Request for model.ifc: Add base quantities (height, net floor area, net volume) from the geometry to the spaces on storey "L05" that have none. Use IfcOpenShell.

First a look at what the model holds.

```python
import ifcopenshell
import ifcopenshell.util.element
import ifcopenshell.util.unit

model = ifcopenshell.open("model.ifc")
print(model.schema)
for unit_type in ("LENGTHUNIT", "AREAUNIT", "VOLUMEUNIT"):
    print(unit_type, ifcopenshell.util.unit.calculate_unit_scale(model, unit_type))
storey = next(s for s in model.by_type("IfcBuildingStorey") if s.Name == "L05")
spaces = [e for e in ifcopenshell.util.element.get_decomposition(storey) if e.is_a("IfcSpace")]
for e in sorted(spaces, key=lambda e: e.id()):
    print(e.id(), e.is_a(), e.Name, list(ifcopenshell.util.element.get_psets(e, qtos_only=True)), sep=" | ")
```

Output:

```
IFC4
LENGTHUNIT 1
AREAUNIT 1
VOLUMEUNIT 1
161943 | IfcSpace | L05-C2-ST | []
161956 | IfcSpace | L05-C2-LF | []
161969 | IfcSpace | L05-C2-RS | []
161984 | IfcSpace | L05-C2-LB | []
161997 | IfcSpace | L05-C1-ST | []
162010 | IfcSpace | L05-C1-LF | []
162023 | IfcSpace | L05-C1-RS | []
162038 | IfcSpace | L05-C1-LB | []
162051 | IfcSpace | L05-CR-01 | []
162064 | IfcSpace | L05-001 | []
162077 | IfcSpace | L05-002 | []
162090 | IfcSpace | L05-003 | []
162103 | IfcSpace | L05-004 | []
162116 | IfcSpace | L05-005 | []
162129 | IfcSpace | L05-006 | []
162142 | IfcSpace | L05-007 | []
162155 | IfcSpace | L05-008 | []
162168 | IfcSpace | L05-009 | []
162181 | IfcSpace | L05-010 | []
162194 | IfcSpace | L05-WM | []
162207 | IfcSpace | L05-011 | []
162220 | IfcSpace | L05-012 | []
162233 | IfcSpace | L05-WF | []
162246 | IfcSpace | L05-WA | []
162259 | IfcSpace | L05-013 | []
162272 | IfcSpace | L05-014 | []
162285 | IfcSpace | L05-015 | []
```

```python
import ifcopenshell
import ifcopenshell.api.pset
import ifcopenshell.geom
import ifcopenshell.util.element
import ifcopenshell.util.shape
import ifcopenshell.util.unit

model = ifcopenshell.open("model.ifc")
unit_scale = ifcopenshell.util.unit.calculate_unit_scale(model)
area_scale = ifcopenshell.util.unit.calculate_unit_scale(model, "AREAUNIT")
volume_scale = ifcopenshell.util.unit.calculate_unit_scale(model, "VOLUMEUNIT")
settings = ifcopenshell.geom.settings()

storey = next(s for s in model.by_type("IfcBuildingStorey") if s.Name == "L05")
spaces = [e for e in ifcopenshell.util.element.get_decomposition(storey) if e.is_a("IfcSpace")]

for e in sorted(spaces, key=lambda e: e.id()):
    if ifcopenshell.util.element.get_psets(e, qtos_only=True, should_inherit=False):
        continue
    # Geometry comes back in metres, in the element's own axes.
    shape = ifcopenshell.geom.create_shape(settings, e)
    values = {
        "Height": ifcopenshell.util.shape.get_z(shape.geometry) / unit_scale,
        "NetFloorArea": ifcopenshell.util.shape.get_footprint_area(shape.geometry) / area_scale,
        "NetVolume": ifcopenshell.util.shape.get_volume(shape.geometry) / volume_scale,
    }
    qto = ifcopenshell.api.pset.add_qto(model, product=e, name="Qto_SpaceBaseQuantities")
    ifcopenshell.api.pset.edit_qto(model, qto=qto, properties=values)
    print(e.id(), {k: round(v, 3) for k, v in values.items()})

model.write("model_v2.ifc")
```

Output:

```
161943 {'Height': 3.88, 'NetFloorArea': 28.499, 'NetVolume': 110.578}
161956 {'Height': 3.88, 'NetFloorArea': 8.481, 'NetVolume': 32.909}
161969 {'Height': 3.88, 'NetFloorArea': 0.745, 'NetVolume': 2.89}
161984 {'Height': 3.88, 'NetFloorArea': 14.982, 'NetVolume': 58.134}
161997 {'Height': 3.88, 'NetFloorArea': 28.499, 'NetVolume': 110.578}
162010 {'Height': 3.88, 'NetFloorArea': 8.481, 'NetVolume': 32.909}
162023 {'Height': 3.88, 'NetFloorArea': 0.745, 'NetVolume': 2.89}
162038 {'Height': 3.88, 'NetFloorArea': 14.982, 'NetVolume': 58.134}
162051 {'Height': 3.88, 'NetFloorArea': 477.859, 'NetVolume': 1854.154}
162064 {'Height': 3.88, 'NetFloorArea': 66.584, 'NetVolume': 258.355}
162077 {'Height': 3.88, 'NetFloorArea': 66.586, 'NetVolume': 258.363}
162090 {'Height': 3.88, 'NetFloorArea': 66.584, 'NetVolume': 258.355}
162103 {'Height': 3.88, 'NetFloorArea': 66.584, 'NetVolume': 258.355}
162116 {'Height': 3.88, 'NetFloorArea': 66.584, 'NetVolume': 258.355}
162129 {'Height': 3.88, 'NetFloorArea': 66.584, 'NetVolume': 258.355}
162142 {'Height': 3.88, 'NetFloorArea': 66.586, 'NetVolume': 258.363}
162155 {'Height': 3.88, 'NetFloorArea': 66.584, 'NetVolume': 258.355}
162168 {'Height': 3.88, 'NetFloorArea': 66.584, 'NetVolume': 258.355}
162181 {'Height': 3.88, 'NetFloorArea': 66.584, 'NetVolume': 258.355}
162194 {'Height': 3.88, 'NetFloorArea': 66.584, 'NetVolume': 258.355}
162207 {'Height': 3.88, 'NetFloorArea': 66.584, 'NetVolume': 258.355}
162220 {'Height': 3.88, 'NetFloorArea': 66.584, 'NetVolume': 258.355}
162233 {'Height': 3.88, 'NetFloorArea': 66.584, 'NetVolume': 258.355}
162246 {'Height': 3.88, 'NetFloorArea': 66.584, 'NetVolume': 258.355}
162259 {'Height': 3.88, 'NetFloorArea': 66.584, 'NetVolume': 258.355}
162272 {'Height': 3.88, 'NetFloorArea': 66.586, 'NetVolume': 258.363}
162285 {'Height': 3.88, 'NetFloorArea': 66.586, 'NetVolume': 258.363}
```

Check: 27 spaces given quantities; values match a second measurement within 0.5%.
